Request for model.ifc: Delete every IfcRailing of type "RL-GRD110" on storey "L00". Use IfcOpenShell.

First a look at what the model holds.

```python
import ifcopenshell
import ifcopenshell.util.element

model = ifcopenshell.open("model.ifc")
print(model.schema)
storey = next(s for s in model.by_type("IfcBuildingStorey") if s.Name == "L00")
railings = [e for e in ifcopenshell.util.element.get_decomposition(storey) if e.is_a("IfcRailing")]
seen = {}
for e in railings:
    element_type = ifcopenshell.util.element.get_type(e)
    name = element_type.Name if element_type not in (None, e) else None
    seen[name] = seen.get(name, 0) + 1
for name, count in sorted(seen.items(), key=str):
    print(count, "x", name)
```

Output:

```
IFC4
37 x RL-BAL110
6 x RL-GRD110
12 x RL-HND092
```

```python
import ifcopenshell
import ifcopenshell.api.root
import ifcopenshell.util.element

model = ifcopenshell.open("model.ifc")

storey = next(s for s in model.by_type("IfcBuildingStorey") if s.Name == "L00")
railings = [e for e in ifcopenshell.util.element.get_decomposition(storey) if e.is_a("IfcRailing")]
targets = [e for e in railings if (t := ifcopenshell.util.element.get_type(e)) not in (None, e) and t.Name == "RL-GRD110"]

for e in targets:
    ifcopenshell.api.root.remove_product(model, product=e)
print(len(targets), "removed")

model.write("model_updated.ifc")
```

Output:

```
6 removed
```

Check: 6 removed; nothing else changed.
